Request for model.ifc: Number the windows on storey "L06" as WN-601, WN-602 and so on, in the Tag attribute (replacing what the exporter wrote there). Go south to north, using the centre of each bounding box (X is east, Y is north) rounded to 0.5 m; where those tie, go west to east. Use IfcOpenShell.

First a look at what the model holds.

```python
import ifcopenshell
import ifcopenshell.util.element
import ifcopenshell.util.placement

model = ifcopenshell.open("model.ifc")
print(model.schema)
storey = next(s for s in model.by_type("IfcBuildingStorey") if s.Name == "L06")
windows = [e for e in ifcopenshell.util.element.get_decomposition(storey) if e.is_a("IfcWindow")]
for e in sorted(windows, key=lambda e: e.id()):
    origin = ifcopenshell.util.placement.get_local_placement(e.ObjectPlacement)[:3, 3]
    print(e.id(), e.Tag, e.Name, origin.round(2) + 0.0, sep=" | ")
```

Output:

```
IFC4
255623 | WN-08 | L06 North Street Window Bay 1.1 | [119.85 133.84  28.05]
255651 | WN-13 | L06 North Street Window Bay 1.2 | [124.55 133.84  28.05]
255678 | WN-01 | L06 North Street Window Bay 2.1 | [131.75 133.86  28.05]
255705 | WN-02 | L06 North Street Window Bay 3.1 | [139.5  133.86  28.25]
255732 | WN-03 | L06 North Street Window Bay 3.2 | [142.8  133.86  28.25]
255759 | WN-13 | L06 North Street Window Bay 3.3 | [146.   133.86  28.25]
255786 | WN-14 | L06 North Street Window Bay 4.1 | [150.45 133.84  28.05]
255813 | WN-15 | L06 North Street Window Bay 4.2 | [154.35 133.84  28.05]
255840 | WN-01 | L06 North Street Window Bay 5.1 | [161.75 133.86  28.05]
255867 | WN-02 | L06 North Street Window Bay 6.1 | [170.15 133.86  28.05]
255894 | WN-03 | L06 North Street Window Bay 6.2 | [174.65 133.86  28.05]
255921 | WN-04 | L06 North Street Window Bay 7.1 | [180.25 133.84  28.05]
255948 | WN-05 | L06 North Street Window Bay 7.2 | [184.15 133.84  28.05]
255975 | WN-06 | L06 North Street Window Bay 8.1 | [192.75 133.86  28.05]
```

```python
import ifcopenshell
import ifcopenshell.geom
import ifcopenshell.util.element
import ifcopenshell.util.shape

model = ifcopenshell.open("model.ifc")
settings = ifcopenshell.geom.settings()
settings.set("use-world-coords", True)


def centre(element):
    shape = ifcopenshell.geom.create_shape(settings, element)
    return ifcopenshell.util.shape.get_bbox_centroid(shape.geometry)


storey = next(s for s in model.by_type("IfcBuildingStorey") if s.Name == "L06")
windows = [e for e in ifcopenshell.util.element.get_decomposition(storey) if e.is_a("IfcWindow")]

# Insertion points can sit at a corner or the storey origin, so sort by the geometry (in metres).
centres = {e: centre(e) for e in windows}
windows.sort(key=lambda e: (round(centres[e][1] / 0.5), centres[e][0]))

for i, e in enumerate(windows, start=1):
    number = f"WN-6{i:02d}"
    e.Tag = number
    print(e.id(), number)

model.write("model_v2.ifc")
```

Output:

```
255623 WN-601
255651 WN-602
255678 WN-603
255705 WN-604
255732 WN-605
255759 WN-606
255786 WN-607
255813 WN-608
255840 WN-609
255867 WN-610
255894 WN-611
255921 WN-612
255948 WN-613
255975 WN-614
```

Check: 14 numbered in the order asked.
